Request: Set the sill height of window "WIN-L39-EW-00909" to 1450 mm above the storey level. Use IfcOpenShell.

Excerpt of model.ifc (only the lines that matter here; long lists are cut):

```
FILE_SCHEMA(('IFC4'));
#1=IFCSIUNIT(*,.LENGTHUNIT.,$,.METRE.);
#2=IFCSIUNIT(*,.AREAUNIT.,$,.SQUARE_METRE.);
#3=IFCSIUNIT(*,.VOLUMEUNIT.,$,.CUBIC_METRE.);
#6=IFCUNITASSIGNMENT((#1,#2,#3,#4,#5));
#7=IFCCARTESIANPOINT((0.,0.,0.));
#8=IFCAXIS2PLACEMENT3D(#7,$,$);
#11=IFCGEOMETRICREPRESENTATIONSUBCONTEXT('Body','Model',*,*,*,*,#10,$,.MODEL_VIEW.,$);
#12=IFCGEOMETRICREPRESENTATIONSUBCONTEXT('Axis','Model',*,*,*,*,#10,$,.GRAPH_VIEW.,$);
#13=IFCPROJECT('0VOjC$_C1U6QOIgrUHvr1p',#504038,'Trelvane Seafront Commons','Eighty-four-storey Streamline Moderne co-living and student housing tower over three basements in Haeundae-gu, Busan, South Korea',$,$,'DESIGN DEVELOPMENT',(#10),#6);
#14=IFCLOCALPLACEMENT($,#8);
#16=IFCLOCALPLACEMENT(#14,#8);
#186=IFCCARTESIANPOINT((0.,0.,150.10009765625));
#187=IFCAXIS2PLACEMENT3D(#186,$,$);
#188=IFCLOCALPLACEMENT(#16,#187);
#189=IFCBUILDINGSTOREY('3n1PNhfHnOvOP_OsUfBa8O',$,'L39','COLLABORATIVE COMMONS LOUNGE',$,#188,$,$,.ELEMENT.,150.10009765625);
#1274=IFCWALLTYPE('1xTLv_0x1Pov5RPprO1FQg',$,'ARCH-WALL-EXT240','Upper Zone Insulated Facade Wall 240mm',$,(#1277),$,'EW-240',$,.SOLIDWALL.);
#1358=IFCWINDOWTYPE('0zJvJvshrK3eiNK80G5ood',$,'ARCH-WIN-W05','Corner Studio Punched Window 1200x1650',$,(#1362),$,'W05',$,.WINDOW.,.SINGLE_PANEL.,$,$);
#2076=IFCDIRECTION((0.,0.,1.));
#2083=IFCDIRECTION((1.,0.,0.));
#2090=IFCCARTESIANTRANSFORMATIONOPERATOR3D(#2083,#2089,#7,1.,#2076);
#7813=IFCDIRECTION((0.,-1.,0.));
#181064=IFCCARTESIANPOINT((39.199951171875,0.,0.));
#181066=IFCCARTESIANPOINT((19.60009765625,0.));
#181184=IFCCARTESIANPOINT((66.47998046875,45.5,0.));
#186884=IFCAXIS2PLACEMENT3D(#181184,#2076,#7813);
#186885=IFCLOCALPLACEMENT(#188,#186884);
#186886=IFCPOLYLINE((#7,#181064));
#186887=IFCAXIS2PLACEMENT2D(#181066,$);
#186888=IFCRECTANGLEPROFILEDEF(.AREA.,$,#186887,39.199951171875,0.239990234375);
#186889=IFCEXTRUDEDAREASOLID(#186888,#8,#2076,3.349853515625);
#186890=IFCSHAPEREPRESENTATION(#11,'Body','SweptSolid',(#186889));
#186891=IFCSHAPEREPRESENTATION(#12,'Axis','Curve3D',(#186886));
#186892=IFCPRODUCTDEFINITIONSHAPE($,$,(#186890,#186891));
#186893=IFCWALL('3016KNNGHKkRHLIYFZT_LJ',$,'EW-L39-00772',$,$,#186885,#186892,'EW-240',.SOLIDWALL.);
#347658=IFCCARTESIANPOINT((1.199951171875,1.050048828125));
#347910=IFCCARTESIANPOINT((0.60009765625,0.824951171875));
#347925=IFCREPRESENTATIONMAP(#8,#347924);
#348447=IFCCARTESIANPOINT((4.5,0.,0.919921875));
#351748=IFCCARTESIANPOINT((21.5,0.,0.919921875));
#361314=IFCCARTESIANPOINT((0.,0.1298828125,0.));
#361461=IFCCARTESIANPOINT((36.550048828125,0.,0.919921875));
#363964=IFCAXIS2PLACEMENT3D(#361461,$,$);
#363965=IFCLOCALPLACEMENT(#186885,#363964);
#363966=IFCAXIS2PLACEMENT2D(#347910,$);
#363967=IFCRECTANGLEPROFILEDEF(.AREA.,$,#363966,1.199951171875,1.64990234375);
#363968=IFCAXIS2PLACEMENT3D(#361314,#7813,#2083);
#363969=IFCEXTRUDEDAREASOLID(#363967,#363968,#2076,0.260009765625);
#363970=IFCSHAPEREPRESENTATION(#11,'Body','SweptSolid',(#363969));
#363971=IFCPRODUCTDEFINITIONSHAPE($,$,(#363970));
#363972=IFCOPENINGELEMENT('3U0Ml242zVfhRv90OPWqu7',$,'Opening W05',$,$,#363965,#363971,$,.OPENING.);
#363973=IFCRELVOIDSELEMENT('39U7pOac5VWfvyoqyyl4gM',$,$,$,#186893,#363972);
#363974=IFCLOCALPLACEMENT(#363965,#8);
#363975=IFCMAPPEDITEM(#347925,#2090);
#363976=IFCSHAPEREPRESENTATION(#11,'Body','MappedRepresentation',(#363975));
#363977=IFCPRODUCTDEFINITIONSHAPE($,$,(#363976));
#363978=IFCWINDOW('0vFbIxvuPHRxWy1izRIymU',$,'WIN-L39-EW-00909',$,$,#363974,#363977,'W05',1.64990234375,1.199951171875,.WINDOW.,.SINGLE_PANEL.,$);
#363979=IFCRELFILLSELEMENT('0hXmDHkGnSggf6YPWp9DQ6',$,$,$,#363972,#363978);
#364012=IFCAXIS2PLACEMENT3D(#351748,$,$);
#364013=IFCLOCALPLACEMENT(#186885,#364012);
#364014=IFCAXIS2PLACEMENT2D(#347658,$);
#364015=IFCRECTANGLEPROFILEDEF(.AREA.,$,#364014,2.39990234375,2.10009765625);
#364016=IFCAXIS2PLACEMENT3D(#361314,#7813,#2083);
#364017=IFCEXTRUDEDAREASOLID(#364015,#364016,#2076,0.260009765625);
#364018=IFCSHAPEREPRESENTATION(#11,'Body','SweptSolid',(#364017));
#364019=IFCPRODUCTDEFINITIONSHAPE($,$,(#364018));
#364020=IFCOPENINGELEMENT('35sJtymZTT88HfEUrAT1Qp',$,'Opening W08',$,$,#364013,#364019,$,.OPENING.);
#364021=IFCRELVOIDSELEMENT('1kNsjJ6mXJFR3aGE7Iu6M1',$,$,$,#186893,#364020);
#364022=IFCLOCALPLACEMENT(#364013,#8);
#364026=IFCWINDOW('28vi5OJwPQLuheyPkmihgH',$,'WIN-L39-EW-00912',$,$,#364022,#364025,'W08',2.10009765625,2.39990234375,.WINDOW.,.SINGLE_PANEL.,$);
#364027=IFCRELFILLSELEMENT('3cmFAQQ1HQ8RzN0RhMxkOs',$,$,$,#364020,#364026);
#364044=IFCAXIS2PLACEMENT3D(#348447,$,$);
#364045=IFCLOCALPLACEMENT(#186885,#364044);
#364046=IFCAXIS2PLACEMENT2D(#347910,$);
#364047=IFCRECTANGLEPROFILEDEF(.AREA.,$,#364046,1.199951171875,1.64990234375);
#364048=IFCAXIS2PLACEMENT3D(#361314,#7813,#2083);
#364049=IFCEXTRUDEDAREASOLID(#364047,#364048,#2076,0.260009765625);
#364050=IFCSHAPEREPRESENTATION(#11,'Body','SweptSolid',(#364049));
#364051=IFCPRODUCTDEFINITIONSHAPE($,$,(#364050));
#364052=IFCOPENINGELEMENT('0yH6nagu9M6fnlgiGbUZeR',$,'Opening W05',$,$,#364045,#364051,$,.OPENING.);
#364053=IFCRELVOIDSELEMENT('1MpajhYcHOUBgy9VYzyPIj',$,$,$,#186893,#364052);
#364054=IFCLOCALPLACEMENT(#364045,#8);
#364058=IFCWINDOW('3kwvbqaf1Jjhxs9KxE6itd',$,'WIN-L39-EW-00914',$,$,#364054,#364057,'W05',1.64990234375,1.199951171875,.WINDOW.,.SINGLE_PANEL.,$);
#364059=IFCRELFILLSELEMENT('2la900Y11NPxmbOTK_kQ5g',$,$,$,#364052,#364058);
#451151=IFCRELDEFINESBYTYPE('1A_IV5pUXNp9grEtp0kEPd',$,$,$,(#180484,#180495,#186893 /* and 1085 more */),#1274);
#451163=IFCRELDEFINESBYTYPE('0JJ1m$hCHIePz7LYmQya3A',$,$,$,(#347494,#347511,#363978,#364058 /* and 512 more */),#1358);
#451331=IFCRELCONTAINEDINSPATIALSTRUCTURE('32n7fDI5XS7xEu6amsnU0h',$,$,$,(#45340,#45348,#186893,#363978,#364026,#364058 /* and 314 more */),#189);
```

```python
import numpy as np
import ifcopenshell
import ifcopenshell.api.geometry
import ifcopenshell.geom
import ifcopenshell.util.element
import ifcopenshell.util.placement
import ifcopenshell.util.shape
import ifcopenshell.util.unit

model = ifcopenshell.open("model.ifc")
unit_scale = ifcopenshell.util.unit.calculate_unit_scale(model)

window = model.by_guid("0vFbIxvuPHRxWy1izRIymU")
opening = window.FillsVoids[0].RelatingOpeningElement
storey = ifcopenshell.util.element.get_container(window, ifc_class="IfcBuildingStorey")
level = ifcopenshell.util.placement.get_local_placement(storey.ObjectPlacement)[2, 3]

# The opening's origin need not be at the sill, so measure its lowest point.
shape = ifcopenshell.geom.create_shape(ifcopenshell.geom.settings(), opening)
bottom = ifcopenshell.util.shape.get_shape_bottom_elevation(shape, shape.geometry) / unit_scale
dz = level + 1.45 - bottom

shift = np.array([0.0, 0.0, dz])
# The window is placed relative to its opening, so it follows when the opening moves.
matrix = ifcopenshell.util.placement.get_local_placement(opening.ObjectPlacement)
matrix[:3, 3] += shift
ifcopenshell.api.geometry.edit_object_placement(
    model, product=opening, matrix=matrix, is_si=False, should_transform_children=True
)

print(f"moved by {dz * unit_scale:+.3f} m")

model.write("model_rev.ifc")
```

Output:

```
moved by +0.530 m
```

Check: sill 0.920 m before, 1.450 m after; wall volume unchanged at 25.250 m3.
